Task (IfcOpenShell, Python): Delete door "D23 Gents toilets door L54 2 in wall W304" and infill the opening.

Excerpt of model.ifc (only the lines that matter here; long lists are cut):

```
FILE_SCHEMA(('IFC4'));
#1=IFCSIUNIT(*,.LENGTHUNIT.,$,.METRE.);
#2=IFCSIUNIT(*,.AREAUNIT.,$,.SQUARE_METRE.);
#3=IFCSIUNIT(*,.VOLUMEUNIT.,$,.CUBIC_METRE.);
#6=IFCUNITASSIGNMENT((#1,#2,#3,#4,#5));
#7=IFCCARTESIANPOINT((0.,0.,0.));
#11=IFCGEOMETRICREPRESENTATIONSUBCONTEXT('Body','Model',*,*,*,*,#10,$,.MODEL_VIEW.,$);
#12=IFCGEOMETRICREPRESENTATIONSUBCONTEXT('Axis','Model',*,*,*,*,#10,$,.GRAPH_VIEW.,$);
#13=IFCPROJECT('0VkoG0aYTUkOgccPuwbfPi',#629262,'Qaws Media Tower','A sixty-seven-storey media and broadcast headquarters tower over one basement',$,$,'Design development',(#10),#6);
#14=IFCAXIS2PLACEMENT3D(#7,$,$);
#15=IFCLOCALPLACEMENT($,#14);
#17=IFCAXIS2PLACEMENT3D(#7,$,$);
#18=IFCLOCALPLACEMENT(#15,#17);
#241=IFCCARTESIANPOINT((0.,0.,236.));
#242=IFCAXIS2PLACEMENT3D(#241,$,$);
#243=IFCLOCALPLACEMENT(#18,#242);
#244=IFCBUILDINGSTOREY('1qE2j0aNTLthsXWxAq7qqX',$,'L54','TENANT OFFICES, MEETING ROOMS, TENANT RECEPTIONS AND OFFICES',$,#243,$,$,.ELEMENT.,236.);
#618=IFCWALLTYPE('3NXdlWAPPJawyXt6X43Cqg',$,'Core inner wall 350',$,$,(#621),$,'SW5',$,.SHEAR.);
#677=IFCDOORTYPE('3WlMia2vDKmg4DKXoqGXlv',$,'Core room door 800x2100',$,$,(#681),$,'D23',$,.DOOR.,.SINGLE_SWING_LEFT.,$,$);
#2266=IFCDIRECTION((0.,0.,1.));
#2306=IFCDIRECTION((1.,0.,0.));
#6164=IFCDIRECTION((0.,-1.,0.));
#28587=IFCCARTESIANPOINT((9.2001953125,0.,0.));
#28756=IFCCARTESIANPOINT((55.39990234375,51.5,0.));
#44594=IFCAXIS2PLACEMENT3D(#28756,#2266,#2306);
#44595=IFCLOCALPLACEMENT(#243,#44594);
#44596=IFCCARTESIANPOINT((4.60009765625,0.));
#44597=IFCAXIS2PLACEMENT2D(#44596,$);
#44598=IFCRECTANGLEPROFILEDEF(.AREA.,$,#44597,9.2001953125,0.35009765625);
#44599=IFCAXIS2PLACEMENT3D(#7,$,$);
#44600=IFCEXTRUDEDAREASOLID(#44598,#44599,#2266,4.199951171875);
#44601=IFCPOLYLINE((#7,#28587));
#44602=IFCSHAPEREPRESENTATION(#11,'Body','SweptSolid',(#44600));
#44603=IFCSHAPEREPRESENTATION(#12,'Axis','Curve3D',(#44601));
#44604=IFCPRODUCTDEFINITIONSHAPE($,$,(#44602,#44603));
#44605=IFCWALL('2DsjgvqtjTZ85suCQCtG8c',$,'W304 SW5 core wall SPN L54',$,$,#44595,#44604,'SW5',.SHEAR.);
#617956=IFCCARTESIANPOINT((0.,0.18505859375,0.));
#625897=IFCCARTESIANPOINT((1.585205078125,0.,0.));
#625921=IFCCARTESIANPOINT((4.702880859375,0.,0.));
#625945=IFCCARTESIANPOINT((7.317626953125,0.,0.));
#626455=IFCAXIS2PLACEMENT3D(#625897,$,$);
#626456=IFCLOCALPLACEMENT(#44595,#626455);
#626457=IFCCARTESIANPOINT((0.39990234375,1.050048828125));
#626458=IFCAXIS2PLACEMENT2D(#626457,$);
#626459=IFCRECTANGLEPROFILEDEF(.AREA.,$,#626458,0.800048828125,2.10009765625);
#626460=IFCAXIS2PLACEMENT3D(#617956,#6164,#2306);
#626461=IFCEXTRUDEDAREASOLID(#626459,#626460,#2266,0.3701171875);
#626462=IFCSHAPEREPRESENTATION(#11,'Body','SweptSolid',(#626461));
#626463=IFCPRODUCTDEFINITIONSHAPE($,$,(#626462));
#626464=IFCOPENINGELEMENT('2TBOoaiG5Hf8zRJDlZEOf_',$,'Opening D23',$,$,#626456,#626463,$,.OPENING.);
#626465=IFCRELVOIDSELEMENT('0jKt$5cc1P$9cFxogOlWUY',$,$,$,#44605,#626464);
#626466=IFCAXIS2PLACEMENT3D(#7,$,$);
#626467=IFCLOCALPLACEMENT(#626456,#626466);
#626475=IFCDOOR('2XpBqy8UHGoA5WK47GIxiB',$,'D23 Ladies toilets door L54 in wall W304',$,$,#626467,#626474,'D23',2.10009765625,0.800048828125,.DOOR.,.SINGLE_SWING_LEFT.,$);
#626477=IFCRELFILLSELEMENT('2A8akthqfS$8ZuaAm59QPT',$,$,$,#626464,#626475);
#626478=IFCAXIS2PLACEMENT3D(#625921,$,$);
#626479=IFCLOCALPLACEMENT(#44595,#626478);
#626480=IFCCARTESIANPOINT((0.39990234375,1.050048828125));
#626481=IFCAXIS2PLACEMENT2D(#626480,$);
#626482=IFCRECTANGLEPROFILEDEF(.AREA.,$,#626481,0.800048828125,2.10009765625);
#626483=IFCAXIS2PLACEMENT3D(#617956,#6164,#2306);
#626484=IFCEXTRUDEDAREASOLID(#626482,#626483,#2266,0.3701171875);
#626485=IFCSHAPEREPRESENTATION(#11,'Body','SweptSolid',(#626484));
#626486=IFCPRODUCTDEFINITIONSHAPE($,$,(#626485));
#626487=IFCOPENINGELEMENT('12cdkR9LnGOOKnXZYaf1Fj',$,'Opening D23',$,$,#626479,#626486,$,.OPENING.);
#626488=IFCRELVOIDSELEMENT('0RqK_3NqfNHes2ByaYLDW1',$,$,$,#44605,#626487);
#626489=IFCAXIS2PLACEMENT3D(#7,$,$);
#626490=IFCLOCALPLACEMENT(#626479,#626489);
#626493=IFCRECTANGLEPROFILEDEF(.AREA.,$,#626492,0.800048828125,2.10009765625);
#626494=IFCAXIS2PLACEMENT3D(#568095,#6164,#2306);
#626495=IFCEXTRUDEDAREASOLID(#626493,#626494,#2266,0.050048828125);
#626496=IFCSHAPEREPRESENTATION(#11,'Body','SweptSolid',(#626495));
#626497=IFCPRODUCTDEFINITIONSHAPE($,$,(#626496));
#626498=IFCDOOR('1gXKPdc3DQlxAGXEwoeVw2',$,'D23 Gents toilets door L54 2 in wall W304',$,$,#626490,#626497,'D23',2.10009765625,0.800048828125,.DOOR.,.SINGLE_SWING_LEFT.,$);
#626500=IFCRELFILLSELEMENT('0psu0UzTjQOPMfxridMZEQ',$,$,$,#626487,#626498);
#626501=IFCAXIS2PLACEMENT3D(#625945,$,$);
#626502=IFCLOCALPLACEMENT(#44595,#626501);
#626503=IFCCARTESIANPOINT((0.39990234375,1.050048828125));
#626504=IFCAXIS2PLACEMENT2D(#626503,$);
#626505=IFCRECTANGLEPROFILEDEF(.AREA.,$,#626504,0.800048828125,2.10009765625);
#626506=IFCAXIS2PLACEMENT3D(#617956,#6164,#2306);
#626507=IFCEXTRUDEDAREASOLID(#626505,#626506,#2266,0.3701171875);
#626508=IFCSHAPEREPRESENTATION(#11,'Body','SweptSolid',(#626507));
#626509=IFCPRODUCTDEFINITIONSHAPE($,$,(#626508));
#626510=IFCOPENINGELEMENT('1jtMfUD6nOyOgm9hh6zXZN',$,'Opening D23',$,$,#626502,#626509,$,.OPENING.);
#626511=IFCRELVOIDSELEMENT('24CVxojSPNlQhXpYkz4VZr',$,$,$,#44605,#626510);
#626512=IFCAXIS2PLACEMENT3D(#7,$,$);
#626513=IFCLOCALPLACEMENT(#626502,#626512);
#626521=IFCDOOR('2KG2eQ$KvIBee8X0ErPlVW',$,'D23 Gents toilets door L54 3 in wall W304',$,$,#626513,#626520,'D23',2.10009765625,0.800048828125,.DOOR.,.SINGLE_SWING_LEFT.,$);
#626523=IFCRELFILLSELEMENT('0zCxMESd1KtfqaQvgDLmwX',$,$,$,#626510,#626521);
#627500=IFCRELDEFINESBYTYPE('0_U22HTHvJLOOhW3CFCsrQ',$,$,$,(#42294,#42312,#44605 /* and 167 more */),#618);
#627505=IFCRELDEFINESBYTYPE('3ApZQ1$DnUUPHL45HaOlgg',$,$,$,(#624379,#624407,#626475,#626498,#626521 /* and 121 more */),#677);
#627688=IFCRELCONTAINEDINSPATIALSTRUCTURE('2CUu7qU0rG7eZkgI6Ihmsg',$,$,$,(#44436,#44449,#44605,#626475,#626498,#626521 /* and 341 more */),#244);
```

```python
import ifcopenshell
import ifcopenshell.api.feature
import ifcopenshell.api.root
import ifcopenshell.geom
import ifcopenshell.util.shape

model = ifcopenshell.open("model.ifc")
settings = ifcopenshell.geom.settings()


def volume(element):
    """Net volume in cubic metres, openings subtracted."""
    shape = ifcopenshell.geom.create_shape(settings, element)
    return ifcopenshell.util.shape.get_volume(shape.geometry)


door = model.by_guid("1gXKPdc3DQlxAGXEwoeVw2")
opening = door.FillsVoids[0].RelatingOpeningElement
wall = opening.VoidsElements[0].RelatingBuildingElement
before = volume(wall)

ifcopenshell.api.root.remove_product(model, product=door)
ifcopenshell.api.feature.remove_feature(model, feature=opening)

after = volume(wall)

print(f"wall volume {before:.3f} -> {after:.3f} m3")

model.write("model_rev.ifc")
```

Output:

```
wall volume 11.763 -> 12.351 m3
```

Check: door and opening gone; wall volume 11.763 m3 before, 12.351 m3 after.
